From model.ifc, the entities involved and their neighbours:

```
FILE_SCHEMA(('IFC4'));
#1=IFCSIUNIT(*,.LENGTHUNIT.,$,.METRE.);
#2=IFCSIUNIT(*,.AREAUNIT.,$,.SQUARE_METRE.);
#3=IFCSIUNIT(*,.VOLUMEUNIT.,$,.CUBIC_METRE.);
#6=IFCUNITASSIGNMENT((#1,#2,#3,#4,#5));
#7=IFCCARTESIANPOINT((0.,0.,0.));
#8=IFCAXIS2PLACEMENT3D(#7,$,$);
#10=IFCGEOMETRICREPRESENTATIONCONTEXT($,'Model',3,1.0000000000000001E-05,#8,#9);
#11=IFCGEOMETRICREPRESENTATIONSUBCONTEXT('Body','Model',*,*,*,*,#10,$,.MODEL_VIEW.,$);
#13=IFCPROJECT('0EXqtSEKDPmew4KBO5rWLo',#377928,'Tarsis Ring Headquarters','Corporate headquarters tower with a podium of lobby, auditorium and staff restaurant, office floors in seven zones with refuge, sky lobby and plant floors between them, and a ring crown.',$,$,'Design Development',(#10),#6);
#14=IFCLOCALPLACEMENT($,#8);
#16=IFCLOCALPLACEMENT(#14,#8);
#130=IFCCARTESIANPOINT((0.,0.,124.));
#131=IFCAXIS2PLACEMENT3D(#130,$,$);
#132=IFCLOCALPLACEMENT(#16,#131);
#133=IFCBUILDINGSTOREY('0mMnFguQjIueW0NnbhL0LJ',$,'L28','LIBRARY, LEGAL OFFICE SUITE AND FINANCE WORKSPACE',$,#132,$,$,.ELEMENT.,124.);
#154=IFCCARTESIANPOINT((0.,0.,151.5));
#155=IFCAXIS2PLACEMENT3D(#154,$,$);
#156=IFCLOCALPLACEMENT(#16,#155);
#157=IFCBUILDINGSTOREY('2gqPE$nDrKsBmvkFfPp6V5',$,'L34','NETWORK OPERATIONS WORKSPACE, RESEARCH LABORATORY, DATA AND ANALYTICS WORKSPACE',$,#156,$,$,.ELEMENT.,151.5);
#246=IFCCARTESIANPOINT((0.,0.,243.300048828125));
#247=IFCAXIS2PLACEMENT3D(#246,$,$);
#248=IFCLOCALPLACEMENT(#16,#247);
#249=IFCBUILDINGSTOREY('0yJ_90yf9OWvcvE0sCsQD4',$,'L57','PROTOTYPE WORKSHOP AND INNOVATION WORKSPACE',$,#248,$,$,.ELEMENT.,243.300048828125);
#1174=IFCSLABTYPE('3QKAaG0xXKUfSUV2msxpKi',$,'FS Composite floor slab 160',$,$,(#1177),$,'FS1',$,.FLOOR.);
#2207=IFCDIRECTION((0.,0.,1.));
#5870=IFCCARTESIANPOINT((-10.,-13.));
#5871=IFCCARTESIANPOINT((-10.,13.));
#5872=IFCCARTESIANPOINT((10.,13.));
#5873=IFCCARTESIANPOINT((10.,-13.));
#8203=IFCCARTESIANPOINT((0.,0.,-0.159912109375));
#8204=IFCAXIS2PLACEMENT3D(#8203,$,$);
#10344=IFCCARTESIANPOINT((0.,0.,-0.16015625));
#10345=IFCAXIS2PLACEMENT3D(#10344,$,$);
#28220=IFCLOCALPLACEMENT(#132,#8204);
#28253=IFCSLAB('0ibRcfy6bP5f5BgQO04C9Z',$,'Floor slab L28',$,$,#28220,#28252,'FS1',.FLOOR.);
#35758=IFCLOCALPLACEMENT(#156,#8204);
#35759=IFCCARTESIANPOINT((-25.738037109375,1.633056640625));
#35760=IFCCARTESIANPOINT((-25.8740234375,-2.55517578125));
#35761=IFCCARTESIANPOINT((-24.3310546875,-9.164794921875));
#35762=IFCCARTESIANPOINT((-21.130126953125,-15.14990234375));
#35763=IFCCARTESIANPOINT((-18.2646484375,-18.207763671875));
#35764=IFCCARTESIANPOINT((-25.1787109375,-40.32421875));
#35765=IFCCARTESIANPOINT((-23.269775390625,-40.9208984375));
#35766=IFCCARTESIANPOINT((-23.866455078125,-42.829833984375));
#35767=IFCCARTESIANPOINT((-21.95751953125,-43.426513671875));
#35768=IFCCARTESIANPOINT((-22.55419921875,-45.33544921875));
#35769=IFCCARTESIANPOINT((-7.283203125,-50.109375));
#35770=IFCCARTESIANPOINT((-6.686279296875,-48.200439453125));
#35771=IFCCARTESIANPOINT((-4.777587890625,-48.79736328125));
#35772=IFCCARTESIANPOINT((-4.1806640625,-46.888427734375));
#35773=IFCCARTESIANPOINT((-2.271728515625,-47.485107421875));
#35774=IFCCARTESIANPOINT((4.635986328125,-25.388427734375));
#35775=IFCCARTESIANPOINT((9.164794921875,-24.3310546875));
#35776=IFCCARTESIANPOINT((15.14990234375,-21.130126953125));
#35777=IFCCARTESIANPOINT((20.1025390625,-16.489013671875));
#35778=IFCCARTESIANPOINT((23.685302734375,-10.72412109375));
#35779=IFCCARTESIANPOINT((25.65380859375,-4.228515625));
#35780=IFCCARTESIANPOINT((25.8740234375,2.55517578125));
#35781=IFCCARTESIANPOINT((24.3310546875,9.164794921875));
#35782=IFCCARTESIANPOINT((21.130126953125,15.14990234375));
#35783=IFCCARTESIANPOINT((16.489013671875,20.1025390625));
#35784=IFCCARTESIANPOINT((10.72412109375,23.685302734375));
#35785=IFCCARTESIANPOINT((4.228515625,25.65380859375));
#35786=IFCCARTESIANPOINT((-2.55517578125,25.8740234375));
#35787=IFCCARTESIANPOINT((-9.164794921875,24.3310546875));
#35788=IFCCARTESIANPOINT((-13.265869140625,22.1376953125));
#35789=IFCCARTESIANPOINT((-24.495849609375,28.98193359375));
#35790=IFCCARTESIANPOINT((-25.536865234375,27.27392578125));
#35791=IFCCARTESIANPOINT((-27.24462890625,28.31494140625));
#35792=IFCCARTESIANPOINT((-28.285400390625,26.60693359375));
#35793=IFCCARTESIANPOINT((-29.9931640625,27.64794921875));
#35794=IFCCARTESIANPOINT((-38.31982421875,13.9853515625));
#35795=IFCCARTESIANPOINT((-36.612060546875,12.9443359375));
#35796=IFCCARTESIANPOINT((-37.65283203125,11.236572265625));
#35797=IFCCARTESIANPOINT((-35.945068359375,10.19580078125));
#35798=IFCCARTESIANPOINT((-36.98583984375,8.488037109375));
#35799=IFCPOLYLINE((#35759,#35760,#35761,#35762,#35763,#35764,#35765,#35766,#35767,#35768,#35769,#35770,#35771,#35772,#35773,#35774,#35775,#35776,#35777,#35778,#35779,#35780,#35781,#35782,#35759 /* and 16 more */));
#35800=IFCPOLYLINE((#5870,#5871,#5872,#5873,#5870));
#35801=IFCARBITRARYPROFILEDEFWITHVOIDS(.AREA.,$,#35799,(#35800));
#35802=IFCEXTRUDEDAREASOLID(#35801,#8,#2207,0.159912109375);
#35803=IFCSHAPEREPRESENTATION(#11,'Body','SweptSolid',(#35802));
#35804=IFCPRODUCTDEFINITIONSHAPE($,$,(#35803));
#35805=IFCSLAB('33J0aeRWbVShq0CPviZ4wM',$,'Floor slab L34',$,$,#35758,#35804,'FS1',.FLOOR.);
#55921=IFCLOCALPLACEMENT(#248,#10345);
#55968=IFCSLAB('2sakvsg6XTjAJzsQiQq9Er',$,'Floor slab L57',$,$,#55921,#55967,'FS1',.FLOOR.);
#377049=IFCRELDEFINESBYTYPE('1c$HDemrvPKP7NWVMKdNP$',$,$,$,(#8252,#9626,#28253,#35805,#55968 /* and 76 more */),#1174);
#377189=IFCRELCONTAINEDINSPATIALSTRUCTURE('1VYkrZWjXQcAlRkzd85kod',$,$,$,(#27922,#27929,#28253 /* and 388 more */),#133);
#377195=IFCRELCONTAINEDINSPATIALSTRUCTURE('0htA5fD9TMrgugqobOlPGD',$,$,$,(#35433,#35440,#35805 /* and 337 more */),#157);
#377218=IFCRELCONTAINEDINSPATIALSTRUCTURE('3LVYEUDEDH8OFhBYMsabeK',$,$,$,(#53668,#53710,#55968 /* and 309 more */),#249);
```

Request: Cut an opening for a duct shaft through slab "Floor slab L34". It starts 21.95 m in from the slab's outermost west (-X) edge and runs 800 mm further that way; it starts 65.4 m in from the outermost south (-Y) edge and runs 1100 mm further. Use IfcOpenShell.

```python
import numpy as np
import ifcopenshell
import ifcopenshell.api.feature
import ifcopenshell.api.geometry
import ifcopenshell.api.root
import ifcopenshell.geom
import ifcopenshell.util.placement
import ifcopenshell.util.representation
import ifcopenshell.util.shape
import ifcopenshell.util.unit

model = ifcopenshell.open("model.ifc")
unit_scale = ifcopenshell.util.unit.calculate_unit_scale(model)
settings = ifcopenshell.geom.settings()


def volume(element):
    """Net volume in cubic metres, openings subtracted."""
    shape = ifcopenshell.geom.create_shape(settings, element)
    return ifcopenshell.util.shape.get_volume(shape.geometry)


slab = model.by_guid("33J0aeRWbVShq0CPviZ4wM")
before = volume(slab)

# Extent in the slab's own axes, in metres. The edges named are its -X and -Y sides.
slab_shape = ifcopenshell.geom.create_shape(settings, slab)
vertices = ifcopenshell.util.shape.get_vertices(slab_shape.geometry)
x_min, y_min, bottom = vertices.min(axis=0)
top = vertices[:, 2].max()

opening = ifcopenshell.api.root.create_entity(model, ifc_class="IfcOpeningElement", name="Duct shaft opening", predefined_type="OPENING")
context = ifcopenshell.util.representation.get_context(model, "Model", "Body", "MODEL_VIEW")
width, depth = 0.8, 1.1
outline = [(0.0, 0.0), (width, 0.0), (width, depth), (0.0, depth), (0.0, 0.0)]
# Overshoot both faces by 50 mm so the cut is clean.
shape = ifcopenshell.api.geometry.add_slab_representation(
    model, context=context, depth=top - bottom + 0.1, polyline=outline
)
ifcopenshell.api.geometry.assign_representation(model, product=opening, representation=shape)

matrix = ifcopenshell.util.placement.get_local_placement(slab.ObjectPlacement)
matrix[:, 3] = matrix @ np.append(np.array([x_min + 21.95, y_min + 65.4, bottom - 0.05]) / unit_scale, 1.0)
ifcopenshell.api.geometry.edit_object_placement(model, product=opening, matrix=matrix, is_si=False)
ifcopenshell.api.feature.add_feature(model, feature=opening, element=slab)

after = volume(slab)

print(f"slab volume {before:.3f} -> {after:.3f} m3")

model.write("model_v2.ifc")
```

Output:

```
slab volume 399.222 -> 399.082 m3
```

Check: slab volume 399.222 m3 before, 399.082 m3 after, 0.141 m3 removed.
